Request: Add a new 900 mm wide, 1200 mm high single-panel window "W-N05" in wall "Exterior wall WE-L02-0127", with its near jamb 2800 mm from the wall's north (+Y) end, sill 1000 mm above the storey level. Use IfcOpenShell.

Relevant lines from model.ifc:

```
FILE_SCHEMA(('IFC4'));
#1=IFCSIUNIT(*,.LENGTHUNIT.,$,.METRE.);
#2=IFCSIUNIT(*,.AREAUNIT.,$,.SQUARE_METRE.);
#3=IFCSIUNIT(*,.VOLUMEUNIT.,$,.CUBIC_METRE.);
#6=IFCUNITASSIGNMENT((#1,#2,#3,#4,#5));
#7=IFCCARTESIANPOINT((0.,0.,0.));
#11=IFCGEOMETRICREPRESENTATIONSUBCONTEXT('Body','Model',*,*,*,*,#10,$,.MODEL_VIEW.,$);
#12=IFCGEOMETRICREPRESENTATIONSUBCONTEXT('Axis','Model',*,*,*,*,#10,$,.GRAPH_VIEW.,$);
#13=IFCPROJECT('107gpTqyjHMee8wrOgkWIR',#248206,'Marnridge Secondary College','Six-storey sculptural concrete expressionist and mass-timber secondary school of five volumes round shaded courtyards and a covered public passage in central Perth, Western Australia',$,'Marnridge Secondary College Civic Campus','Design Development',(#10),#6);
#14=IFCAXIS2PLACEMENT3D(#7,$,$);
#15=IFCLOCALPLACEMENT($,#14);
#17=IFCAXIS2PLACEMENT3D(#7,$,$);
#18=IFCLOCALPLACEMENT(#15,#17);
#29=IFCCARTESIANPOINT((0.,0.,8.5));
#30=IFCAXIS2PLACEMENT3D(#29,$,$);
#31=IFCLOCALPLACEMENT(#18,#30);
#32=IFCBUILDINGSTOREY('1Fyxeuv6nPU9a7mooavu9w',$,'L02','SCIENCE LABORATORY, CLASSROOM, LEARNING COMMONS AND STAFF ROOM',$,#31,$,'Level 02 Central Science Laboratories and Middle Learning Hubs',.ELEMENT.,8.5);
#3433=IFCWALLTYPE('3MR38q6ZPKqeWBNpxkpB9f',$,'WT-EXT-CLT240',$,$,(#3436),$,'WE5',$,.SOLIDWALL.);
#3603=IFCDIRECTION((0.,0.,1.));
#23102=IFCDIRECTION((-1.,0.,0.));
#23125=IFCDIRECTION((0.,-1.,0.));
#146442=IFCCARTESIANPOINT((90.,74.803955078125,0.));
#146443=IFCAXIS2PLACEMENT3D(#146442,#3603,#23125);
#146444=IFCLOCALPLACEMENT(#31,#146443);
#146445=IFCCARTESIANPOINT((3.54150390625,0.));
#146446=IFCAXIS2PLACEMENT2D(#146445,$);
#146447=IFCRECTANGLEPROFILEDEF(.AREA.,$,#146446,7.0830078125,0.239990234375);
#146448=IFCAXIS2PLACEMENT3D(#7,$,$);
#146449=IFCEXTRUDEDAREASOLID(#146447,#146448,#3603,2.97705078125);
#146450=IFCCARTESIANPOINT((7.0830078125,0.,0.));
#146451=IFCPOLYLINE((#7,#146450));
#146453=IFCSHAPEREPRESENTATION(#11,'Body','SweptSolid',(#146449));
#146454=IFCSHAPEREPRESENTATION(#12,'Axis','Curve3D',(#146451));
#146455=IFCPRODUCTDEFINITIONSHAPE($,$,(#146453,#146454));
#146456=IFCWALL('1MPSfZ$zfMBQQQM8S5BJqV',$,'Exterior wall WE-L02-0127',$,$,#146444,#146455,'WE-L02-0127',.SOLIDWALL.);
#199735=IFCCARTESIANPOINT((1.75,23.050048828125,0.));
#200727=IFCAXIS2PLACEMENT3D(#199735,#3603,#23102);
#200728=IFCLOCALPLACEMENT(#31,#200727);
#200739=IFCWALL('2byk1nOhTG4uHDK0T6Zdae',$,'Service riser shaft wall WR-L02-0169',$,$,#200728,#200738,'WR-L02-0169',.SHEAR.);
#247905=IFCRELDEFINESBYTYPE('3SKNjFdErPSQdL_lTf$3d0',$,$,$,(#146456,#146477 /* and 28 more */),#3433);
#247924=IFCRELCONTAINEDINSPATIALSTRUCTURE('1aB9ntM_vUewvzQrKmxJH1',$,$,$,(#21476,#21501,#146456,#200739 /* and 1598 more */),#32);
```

```python
import numpy as np
import ifcopenshell
import ifcopenshell.api.feature
import ifcopenshell.api.geometry
import ifcopenshell.api.root
import ifcopenshell.api.spatial
import ifcopenshell.geom
import ifcopenshell.util.element
import ifcopenshell.util.placement
import ifcopenshell.util.representation
import ifcopenshell.util.shape
import ifcopenshell.util.unit

model = ifcopenshell.open("model.ifc")
unit_scale = ifcopenshell.util.unit.calculate_unit_scale(model)
settings = ifcopenshell.geom.settings()


def volume(element):
    """Net volume in cubic metres, openings subtracted."""
    shape = ifcopenshell.geom.create_shape(settings, element)
    return ifcopenshell.util.shape.get_volume(shape.geometry)


wall = model.by_guid("1MPSfZ$zfMBQQQM8S5BJqV")
storey = ifcopenshell.util.element.get_container(wall, ifc_class="IfcBuildingStorey")
context = ifcopenshell.util.representation.get_context(model, "Model", "Body", "MODEL_VIEW")
before = volume(wall)

width, height, from_end, sill = 0.9, 1.2, 2.8, 1  # metres

# The wall runs along its own X axis, and the end named is its -X end.
wall_shape = ifcopenshell.geom.create_shape(settings, wall)
x, y, z = ifcopenshell.util.shape.get_vertices(wall_shape.geometry).T
start = x.min() + from_end
face, thickness = float(y.min()), float(y.max() - y.min())
wall_matrix = ifcopenshell.util.placement.get_local_placement(wall.ObjectPlacement)
level = ifcopenshell.util.placement.get_local_placement(storey.ObjectPlacement)[2, 3]


def in_wall(x, y):
    """Placement at x, y metres in the wall's axes, at sill height."""
    matrix = wall_matrix.copy()
    matrix[:, 3] = wall_matrix @ np.array([x / unit_scale, y / unit_scale, 0.0, 1.0])
    matrix[2, 3] = level + sill / unit_scale
    return matrix


# Opening: a box that overshoots both wall faces by 50 mm.
opening = ifcopenshell.api.root.create_entity(model, ifc_class="IfcOpeningElement", predefined_type="OPENING")
box = ifcopenshell.api.geometry.add_wall_representation(
    model, context=context, length=width, height=height, thickness=thickness + 0.1
)
ifcopenshell.api.geometry.assign_representation(model, product=opening, representation=box)
ifcopenshell.api.geometry.edit_object_placement(model, product=opening, matrix=in_wall(start, face - 0.05), is_si=False)
ifcopenshell.api.feature.add_feature(model, feature=opening, element=wall)

window = ifcopenshell.api.root.create_entity(model, ifc_class="IfcWindow", name="W-N05", predefined_type="WINDOW")
window.OverallWidth, window.OverallHeight = width / unit_scale, height / unit_scale
window.PartitioningType = "SINGLE_PANEL"
body = ifcopenshell.api.geometry.add_window_representation(
    model,
    context=context,
    overall_width=window.OverallWidth,
    overall_height=window.OverallHeight,
    partition_type="SINGLE_PANEL",
)
ifcopenshell.api.geometry.assign_representation(model, product=window, representation=body)
ifcopenshell.api.spatial.assign_container(model, products=[window], relating_structure=storey)
ifcopenshell.api.feature.add_filling(model, opening=opening, element=window)

# Centre the window in the wall's thickness.
ifcopenshell.api.geometry.edit_object_placement(model, product=window, matrix=in_wall(start, face), is_si=False)
window_shape = ifcopenshell.geom.create_shape(settings, window)
depth = ifcopenshell.util.shape.get_vertices(window_shape.geometry)[:, 1]
offset = face + thickness / 2 - (depth.min() + depth.max()) / 2
ifcopenshell.api.geometry.edit_object_placement(model, product=window, matrix=in_wall(start, offset), is_si=False)

after = volume(wall)

print(f"wall volume {before:.3f} -> {after:.3f} m3")

model.write("model_v2.ifc")
```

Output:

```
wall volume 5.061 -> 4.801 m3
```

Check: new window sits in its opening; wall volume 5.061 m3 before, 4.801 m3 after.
